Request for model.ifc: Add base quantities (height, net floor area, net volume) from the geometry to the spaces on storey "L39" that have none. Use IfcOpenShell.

First a look at what the model holds.

```python
import ifcopenshell
import ifcopenshell.util.element
import ifcopenshell.util.unit

model = ifcopenshell.open("model.ifc")
print(model.schema)
for unit_type in ("LENGTHUNIT", "AREAUNIT", "VOLUMEUNIT"):
    print(unit_type, ifcopenshell.util.unit.calculate_unit_scale(model, unit_type))
storey = next(s for s in model.by_type("IfcBuildingStorey") if s.Name == "L39")
spaces = [e for e in ifcopenshell.util.element.get_decomposition(storey) if e.is_a("IfcSpace")]
for e in sorted(spaces, key=lambda e: e.id()):
    print(e.id(), e.is_a(), e.Name, list(ifcopenshell.util.element.get_psets(e, qtos_only=True)), sep=" | ")
```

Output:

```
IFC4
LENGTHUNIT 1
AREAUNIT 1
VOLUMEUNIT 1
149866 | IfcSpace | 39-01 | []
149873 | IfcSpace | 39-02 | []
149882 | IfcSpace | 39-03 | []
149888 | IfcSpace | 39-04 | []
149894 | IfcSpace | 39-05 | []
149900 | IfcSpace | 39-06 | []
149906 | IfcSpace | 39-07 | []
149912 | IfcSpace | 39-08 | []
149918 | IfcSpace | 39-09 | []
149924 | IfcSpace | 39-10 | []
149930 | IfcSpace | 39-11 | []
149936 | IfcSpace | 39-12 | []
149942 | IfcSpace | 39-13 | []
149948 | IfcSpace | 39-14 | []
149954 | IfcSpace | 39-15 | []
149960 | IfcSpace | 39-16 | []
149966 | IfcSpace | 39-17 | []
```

```python
import ifcopenshell
import ifcopenshell.api.pset
import ifcopenshell.geom
import ifcopenshell.util.element
import ifcopenshell.util.shape
import ifcopenshell.util.unit

model = ifcopenshell.open("model.ifc")
unit_scale = ifcopenshell.util.unit.calculate_unit_scale(model)
area_scale = ifcopenshell.util.unit.calculate_unit_scale(model, "AREAUNIT")
volume_scale = ifcopenshell.util.unit.calculate_unit_scale(model, "VOLUMEUNIT")
settings = ifcopenshell.geom.settings()

storey = next(s for s in model.by_type("IfcBuildingStorey") if s.Name == "L39")
spaces = [e for e in ifcopenshell.util.element.get_decomposition(storey) if e.is_a("IfcSpace")]

for e in sorted(spaces, key=lambda e: e.id()):
    if ifcopenshell.util.element.get_psets(e, qtos_only=True, should_inherit=False):
        continue
    # Geometry comes back in metres, in the element's own axes.
    shape = ifcopenshell.geom.create_shape(settings, e)
    values = {
        "Height": ifcopenshell.util.shape.get_z(shape.geometry) / unit_scale,
        "NetFloorArea": ifcopenshell.util.shape.get_footprint_area(shape.geometry) / area_scale,
        "NetVolume": ifcopenshell.util.shape.get_volume(shape.geometry) / volume_scale,
    }
    qto = ifcopenshell.api.pset.add_qto(model, product=e, name="Qto_SpaceBaseQuantities")
    ifcopenshell.api.pset.edit_qto(model, qto=qto, properties=values)
    print(e.id(), {k: round(v, 3) for k, v in values.items()})

model.write("model_updated.ifc")
```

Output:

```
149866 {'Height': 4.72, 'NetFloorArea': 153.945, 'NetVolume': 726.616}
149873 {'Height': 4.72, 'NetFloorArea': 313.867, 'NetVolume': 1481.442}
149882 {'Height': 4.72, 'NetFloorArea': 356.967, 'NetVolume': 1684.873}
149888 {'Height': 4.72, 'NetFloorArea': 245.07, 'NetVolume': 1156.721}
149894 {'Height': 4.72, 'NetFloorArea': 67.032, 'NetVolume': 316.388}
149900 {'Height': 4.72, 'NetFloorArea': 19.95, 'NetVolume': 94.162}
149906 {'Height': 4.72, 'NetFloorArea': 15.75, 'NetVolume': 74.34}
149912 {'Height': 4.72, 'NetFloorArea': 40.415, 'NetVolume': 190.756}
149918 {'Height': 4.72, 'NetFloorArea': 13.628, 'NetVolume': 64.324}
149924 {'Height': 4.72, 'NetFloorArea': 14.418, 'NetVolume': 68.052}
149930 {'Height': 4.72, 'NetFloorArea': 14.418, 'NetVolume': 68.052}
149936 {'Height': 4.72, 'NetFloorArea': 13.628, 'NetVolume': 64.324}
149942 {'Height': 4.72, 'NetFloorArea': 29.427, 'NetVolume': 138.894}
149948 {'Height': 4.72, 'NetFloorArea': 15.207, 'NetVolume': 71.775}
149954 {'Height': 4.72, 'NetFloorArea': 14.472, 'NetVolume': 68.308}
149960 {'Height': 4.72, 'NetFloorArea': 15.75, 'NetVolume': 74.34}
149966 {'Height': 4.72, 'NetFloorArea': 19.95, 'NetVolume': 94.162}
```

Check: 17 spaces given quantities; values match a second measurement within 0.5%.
